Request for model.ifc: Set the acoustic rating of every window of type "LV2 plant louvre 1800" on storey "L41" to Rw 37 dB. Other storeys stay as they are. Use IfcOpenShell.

First a look at what the model holds.

```python
import ifcopenshell
import ifcopenshell.util.element

model = ifcopenshell.open("model.ifc")
print(model.schema)
storey = next(s for s in model.by_type("IfcBuildingStorey") if s.Name == "L41")
windows = [e for e in ifcopenshell.util.element.get_decomposition(storey) if e.is_a("IfcWindow")]
seen = {}
for e in windows:
    element_type = ifcopenshell.util.element.get_type(e)
    key = (element_type.Name if element_type != e and element_type else None, ifcopenshell.util.element.get_pset(e, "Pset_WindowCommon", "AcousticRating"))
    seen[key] = seen.get(key, 0) + 1
for (name, value), count in sorted(seen.items(), key=str):
    print(count, "x", name, "|", value)
```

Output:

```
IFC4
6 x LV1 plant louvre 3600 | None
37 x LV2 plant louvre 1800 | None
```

```python
import ifcopenshell
import ifcopenshell.api.pset
import ifcopenshell.util.element

model = ifcopenshell.open("model.ifc")

storey = next(s for s in model.by_type("IfcBuildingStorey") if s.Name == "L41")
windows = [e for e in ifcopenshell.util.element.get_decomposition(storey) if e.is_a("IfcWindow")]

count = 0
for e in windows:
    element_type = ifcopenshell.util.element.get_type(e)
    if element_type in (None, e) or element_type.Name != "LV2 plant louvre 1800":
        continue
    found = ifcopenshell.util.element.get_pset(e, "Pset_WindowCommon", should_inherit=False)
    if found:
        pset = model.by_id(found["id"])
        if len(ifcopenshell.util.element.get_elements_by_pset(pset)) > 1:
            pset = ifcopenshell.api.pset.unshare_pset(model, products=[e], pset=pset)[0]
    else:
        pset = ifcopenshell.api.pset.add_pset(model, product=e, name="Pset_WindowCommon")
    ifcopenshell.api.pset.edit_pset(model, pset=pset, properties={"AcousticRating": "Rw 37 dB"})
    count += 1

print(count, "windows updated")

model.write("model_rev.ifc")
```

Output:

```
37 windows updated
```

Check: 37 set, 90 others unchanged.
